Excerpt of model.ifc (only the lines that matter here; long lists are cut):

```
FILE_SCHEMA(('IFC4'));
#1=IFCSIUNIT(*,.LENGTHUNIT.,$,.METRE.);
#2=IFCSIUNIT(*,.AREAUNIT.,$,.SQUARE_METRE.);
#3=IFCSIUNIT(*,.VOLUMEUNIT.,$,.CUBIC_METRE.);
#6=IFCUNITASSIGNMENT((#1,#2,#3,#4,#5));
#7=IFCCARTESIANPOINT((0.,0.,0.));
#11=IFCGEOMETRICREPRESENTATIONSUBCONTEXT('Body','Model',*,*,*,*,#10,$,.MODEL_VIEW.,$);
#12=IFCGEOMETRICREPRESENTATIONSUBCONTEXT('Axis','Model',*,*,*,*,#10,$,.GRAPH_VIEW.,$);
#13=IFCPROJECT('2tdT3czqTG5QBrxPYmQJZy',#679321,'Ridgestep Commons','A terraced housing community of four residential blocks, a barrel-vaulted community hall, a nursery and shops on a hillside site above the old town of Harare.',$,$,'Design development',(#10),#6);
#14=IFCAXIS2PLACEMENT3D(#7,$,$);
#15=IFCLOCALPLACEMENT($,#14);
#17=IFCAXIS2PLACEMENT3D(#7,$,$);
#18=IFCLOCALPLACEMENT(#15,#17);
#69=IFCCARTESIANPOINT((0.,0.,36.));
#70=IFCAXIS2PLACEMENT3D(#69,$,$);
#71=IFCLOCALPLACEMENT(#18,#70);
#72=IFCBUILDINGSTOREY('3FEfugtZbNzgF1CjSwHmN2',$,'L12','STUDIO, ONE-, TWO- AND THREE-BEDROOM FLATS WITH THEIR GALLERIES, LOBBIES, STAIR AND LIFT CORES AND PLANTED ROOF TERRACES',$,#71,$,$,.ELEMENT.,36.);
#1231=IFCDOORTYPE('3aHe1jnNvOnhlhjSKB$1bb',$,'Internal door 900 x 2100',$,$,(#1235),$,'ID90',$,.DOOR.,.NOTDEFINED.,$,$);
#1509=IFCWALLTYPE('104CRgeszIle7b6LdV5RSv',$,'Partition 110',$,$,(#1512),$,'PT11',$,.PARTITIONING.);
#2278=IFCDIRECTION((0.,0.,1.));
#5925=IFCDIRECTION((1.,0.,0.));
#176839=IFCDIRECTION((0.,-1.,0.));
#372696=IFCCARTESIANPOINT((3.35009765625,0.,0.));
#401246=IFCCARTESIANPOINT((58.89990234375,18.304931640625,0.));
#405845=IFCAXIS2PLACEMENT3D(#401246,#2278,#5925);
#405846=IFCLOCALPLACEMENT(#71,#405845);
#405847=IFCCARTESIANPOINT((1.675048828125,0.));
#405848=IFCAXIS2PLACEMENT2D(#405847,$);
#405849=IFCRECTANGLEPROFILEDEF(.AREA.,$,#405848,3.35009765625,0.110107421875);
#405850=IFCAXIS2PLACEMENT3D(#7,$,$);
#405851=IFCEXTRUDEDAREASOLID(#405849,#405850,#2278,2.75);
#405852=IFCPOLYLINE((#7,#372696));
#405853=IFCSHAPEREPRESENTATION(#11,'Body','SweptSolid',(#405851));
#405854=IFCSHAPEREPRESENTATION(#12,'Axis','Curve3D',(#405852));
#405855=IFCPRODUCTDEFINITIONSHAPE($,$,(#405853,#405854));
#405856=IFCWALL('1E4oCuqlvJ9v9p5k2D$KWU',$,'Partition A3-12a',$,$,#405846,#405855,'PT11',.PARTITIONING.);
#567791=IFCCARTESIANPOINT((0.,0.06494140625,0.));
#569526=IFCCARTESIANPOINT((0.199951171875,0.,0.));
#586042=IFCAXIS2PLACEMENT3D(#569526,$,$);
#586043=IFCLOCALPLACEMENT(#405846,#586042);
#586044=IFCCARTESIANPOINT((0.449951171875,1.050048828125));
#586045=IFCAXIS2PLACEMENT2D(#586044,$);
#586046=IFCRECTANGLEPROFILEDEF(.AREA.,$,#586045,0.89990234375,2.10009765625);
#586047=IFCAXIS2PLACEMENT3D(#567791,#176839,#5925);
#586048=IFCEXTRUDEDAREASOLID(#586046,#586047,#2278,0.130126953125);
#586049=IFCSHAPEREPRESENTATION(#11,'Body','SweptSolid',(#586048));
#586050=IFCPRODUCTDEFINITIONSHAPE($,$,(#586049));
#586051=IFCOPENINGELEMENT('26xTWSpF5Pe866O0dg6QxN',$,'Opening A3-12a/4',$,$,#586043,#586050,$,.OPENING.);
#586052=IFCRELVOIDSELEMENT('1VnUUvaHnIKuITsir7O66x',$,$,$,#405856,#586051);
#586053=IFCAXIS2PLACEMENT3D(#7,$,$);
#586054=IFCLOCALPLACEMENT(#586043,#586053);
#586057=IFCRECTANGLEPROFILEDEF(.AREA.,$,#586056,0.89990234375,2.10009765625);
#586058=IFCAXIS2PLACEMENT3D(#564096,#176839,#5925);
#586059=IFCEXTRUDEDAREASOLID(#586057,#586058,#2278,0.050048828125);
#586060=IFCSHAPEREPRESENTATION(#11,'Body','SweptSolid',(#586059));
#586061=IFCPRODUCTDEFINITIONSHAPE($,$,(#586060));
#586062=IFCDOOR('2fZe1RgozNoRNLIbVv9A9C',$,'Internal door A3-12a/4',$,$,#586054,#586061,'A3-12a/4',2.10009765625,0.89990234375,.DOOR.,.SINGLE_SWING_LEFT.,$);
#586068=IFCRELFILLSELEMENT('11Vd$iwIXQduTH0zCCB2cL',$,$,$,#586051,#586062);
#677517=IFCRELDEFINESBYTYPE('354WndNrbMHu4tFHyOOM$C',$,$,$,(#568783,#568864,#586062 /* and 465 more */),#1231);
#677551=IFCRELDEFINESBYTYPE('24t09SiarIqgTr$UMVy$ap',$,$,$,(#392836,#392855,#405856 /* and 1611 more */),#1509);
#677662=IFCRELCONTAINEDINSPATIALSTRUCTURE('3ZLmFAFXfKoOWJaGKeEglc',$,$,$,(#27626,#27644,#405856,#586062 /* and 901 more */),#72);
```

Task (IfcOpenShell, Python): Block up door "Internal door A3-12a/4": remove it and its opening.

```python
import ifcopenshell
import ifcopenshell.api.feature
import ifcopenshell.api.root
import ifcopenshell.geom
import ifcopenshell.util.shape

model = ifcopenshell.open("model.ifc")
settings = ifcopenshell.geom.settings()


def volume(element):
    """Net volume in cubic metres, openings subtracted."""
    shape = ifcopenshell.geom.create_shape(settings, element)
    return ifcopenshell.util.shape.get_volume(shape.geometry)


door = model.by_guid("2fZe1RgozNoRNLIbVv9A9C")
opening = door.FillsVoids[0].RelatingOpeningElement
wall = opening.VoidsElements[0].RelatingBuildingElement
before = volume(wall)

ifcopenshell.api.root.remove_product(model, product=door)
ifcopenshell.api.feature.remove_feature(model, feature=opening)

after = volume(wall)

print(f"wall volume {before:.3f} -> {after:.3f} m3")

model.write("model-out.ifc")
```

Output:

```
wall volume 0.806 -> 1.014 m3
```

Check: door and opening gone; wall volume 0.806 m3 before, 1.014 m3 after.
